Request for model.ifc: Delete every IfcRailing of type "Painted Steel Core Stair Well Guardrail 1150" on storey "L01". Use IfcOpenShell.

First a look at what the model holds.

```python
import ifcopenshell
import ifcopenshell.util.element

model = ifcopenshell.open("model.ifc")
print(model.schema)
storey = next(s for s in model.by_type("IfcBuildingStorey") if s.Name == "L01")
railings = [e for e in ifcopenshell.util.element.get_decomposition(storey) if e.is_a("IfcRailing")]
seen = {}
for e in railings:
    element_type = ifcopenshell.util.element.get_type(e)
    name = element_type.Name if element_type not in (None, e) else None
    seen[name] = seen.get(name, 0) + 1
for name, count in sorted(seen.items(), key=str):
    print(count, "x", name)
```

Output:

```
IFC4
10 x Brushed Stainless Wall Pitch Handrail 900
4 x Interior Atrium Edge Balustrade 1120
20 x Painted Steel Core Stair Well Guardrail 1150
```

```python
import ifcopenshell
import ifcopenshell.api.root
import ifcopenshell.util.element

model = ifcopenshell.open("model.ifc")

storey = next(s for s in model.by_type("IfcBuildingStorey") if s.Name == "L01")
railings = [e for e in ifcopenshell.util.element.get_decomposition(storey) if e.is_a("IfcRailing")]
targets = [e for e in railings if (t := ifcopenshell.util.element.get_type(e)) not in (None, e) and t.Name == "Painted Steel Core Stair Well Guardrail 1150"]

for e in targets:
    ifcopenshell.api.root.remove_product(model, product=e)
print(len(targets), "removed")

model.write("model_v2.ifc")
```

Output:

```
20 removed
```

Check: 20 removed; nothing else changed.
